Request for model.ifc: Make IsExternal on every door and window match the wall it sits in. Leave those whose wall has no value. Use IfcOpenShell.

First a look at what the model holds.

```python
import ifcopenshell
import ifcopenshell.util.element

model = ifcopenshell.open("model.ifc")
print(model.schema)
seen = {}
for e in model.by_type("IfcDoor") + model.by_type("IfcWindow"):
    if not e.FillsVoids:
        continue
    host = e.FillsVoids[0].RelatingOpeningElement.VoidsElements[0].RelatingBuildingElement
    own = ifcopenshell.util.element.get_pset(e, f"Pset_{e.is_a()[3:].removesuffix('StandardCase')}Common", "IsExternal")
    wall = ifcopenshell.util.element.get_pset(host, "Pset_WallCommon", "IsExternal")
    seen[e.is_a(), own, wall] = seen.get((e.is_a(), own, wall), 0) + 1
for (cls, own, wall), count in sorted(seen.items(), key=str):
    print(count, cls, "IsExternal:", own, "| host wall:", wall)
```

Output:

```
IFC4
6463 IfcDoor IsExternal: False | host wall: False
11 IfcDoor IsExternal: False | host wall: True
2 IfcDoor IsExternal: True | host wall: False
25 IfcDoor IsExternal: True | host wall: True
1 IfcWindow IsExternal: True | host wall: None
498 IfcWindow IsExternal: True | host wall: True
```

```python
import ifcopenshell
import ifcopenshell.api.pset
import ifcopenshell.util.element

model = ifcopenshell.open("model.ifc")

count = 0
for ifc_class, pset_name in (("IfcDoor", "Pset_DoorCommon"), ("IfcWindow", "Pset_WindowCommon")):
    for e in model.by_type(ifc_class):
        if not e.FillsVoids:
            continue
        host = e.FillsVoids[0].RelatingOpeningElement.VoidsElements[0].RelatingBuildingElement
        external = ifcopenshell.util.element.get_pset(host, "Pset_WallCommon", "IsExternal")
        if external is None or ifcopenshell.util.element.get_pset(e, pset_name, "IsExternal") == external:
            continue
        found = ifcopenshell.util.element.get_pset(e, pset_name, should_inherit=False)
        if found:
            pset = model.by_id(found["id"])
            if len(ifcopenshell.util.element.get_elements_by_pset(pset)) > 1:
                pset = ifcopenshell.api.pset.unshare_pset(model, products=[e], pset=pset)[0]
        else:
            pset = ifcopenshell.api.pset.add_pset(model, product=e, name=pset_name)
        ifcopenshell.api.pset.edit_pset(model, pset=pset, properties={"IsExternal": external})
        count += 1

print(count, "updated")

model.write("model_rev.ifc")
```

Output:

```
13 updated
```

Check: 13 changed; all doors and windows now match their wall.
